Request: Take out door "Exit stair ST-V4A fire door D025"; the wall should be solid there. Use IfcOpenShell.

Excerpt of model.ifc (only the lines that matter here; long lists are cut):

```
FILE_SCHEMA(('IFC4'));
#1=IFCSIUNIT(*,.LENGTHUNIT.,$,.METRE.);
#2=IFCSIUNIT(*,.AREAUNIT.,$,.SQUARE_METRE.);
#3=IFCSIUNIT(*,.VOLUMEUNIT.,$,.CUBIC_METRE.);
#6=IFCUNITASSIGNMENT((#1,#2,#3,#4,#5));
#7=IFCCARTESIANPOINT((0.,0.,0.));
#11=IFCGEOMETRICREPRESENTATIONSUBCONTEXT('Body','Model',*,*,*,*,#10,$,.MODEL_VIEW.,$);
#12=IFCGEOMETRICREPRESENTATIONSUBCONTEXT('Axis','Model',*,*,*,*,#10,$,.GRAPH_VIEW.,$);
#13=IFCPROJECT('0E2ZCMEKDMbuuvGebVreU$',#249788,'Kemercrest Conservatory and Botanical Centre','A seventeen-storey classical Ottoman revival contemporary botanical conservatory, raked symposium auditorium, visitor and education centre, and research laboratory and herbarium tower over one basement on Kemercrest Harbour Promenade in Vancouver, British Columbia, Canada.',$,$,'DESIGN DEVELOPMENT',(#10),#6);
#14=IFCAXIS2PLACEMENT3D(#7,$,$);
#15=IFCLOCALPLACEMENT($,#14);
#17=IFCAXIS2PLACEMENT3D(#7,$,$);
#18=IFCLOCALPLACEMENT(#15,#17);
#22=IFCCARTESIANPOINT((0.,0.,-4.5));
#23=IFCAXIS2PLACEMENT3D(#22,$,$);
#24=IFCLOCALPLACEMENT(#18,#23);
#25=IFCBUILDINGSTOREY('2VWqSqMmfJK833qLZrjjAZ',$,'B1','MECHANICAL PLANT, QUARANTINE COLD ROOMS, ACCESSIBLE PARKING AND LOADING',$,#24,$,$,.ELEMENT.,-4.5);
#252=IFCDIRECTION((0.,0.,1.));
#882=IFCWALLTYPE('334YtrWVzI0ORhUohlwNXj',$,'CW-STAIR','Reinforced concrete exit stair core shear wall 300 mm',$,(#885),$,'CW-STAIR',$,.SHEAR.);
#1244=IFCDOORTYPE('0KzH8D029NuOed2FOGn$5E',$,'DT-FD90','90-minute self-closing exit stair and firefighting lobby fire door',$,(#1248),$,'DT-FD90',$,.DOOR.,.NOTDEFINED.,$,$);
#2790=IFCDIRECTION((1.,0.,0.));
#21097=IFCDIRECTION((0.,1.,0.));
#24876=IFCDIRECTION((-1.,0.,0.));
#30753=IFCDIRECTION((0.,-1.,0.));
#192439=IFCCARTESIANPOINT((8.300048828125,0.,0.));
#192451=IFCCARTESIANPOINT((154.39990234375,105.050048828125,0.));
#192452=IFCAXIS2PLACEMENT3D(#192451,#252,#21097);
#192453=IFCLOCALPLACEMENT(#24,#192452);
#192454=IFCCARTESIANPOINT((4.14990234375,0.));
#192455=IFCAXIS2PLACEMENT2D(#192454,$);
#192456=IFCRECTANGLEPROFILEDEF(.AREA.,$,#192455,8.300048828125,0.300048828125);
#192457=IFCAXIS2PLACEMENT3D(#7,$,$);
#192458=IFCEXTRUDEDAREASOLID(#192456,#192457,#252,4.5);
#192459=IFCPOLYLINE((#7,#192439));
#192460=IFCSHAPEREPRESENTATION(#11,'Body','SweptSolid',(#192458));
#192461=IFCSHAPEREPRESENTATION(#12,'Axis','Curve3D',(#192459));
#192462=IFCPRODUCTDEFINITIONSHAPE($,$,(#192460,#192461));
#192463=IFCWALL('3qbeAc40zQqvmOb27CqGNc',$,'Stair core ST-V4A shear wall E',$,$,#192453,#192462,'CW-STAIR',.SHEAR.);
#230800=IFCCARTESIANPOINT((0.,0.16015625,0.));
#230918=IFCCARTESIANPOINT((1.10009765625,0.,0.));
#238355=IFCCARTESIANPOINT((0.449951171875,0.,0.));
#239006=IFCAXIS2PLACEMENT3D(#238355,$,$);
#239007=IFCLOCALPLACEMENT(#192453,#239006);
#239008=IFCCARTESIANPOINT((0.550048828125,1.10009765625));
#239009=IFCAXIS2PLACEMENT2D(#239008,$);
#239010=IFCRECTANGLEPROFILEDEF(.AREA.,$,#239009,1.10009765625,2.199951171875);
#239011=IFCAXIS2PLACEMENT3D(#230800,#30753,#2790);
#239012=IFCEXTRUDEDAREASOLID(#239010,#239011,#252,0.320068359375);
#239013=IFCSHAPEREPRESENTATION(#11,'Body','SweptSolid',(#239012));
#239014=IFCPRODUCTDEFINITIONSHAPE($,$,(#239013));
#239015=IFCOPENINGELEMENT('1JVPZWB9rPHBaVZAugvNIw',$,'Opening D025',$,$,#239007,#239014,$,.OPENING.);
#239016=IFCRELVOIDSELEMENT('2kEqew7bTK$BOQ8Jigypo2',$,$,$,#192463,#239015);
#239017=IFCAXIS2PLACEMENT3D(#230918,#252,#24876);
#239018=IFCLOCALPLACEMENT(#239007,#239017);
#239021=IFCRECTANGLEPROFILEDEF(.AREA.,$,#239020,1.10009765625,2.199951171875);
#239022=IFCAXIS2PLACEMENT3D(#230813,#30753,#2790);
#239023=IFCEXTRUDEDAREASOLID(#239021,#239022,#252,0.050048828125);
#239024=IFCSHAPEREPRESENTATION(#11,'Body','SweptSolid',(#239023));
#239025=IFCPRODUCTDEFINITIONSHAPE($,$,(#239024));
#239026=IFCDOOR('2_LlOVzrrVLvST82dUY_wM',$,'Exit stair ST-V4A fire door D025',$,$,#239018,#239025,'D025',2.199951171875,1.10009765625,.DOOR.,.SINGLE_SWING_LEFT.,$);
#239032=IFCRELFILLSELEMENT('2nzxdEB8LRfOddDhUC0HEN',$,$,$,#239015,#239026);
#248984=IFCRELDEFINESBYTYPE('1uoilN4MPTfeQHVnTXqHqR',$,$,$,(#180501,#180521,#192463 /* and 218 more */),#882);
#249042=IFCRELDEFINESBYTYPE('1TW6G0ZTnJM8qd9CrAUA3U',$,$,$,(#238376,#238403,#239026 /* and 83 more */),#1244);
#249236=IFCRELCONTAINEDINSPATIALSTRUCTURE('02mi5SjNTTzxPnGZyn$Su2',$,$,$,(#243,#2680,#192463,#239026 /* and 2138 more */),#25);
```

```python
import ifcopenshell
import ifcopenshell.api.feature
import ifcopenshell.api.root
import ifcopenshell.geom
import ifcopenshell.util.shape

model = ifcopenshell.open("model.ifc")
settings = ifcopenshell.geom.settings()


def volume(element):
    """Net volume in cubic metres, openings subtracted."""
    shape = ifcopenshell.geom.create_shape(settings, element)
    return ifcopenshell.util.shape.get_volume(shape.geometry)


door = model.by_guid("2_LlOVzrrVLvST82dUY_wM")
opening = door.FillsVoids[0].RelatingOpeningElement
wall = opening.VoidsElements[0].RelatingBuildingElement
before = volume(wall)

ifcopenshell.api.root.remove_product(model, product=door)
ifcopenshell.api.feature.remove_feature(model, feature=opening)

after = volume(wall)

print(f"wall volume {before:.3f} -> {after:.3f} m3")

model.write("model_updated.ifc")
```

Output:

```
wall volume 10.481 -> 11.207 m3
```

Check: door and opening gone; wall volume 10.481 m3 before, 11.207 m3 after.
